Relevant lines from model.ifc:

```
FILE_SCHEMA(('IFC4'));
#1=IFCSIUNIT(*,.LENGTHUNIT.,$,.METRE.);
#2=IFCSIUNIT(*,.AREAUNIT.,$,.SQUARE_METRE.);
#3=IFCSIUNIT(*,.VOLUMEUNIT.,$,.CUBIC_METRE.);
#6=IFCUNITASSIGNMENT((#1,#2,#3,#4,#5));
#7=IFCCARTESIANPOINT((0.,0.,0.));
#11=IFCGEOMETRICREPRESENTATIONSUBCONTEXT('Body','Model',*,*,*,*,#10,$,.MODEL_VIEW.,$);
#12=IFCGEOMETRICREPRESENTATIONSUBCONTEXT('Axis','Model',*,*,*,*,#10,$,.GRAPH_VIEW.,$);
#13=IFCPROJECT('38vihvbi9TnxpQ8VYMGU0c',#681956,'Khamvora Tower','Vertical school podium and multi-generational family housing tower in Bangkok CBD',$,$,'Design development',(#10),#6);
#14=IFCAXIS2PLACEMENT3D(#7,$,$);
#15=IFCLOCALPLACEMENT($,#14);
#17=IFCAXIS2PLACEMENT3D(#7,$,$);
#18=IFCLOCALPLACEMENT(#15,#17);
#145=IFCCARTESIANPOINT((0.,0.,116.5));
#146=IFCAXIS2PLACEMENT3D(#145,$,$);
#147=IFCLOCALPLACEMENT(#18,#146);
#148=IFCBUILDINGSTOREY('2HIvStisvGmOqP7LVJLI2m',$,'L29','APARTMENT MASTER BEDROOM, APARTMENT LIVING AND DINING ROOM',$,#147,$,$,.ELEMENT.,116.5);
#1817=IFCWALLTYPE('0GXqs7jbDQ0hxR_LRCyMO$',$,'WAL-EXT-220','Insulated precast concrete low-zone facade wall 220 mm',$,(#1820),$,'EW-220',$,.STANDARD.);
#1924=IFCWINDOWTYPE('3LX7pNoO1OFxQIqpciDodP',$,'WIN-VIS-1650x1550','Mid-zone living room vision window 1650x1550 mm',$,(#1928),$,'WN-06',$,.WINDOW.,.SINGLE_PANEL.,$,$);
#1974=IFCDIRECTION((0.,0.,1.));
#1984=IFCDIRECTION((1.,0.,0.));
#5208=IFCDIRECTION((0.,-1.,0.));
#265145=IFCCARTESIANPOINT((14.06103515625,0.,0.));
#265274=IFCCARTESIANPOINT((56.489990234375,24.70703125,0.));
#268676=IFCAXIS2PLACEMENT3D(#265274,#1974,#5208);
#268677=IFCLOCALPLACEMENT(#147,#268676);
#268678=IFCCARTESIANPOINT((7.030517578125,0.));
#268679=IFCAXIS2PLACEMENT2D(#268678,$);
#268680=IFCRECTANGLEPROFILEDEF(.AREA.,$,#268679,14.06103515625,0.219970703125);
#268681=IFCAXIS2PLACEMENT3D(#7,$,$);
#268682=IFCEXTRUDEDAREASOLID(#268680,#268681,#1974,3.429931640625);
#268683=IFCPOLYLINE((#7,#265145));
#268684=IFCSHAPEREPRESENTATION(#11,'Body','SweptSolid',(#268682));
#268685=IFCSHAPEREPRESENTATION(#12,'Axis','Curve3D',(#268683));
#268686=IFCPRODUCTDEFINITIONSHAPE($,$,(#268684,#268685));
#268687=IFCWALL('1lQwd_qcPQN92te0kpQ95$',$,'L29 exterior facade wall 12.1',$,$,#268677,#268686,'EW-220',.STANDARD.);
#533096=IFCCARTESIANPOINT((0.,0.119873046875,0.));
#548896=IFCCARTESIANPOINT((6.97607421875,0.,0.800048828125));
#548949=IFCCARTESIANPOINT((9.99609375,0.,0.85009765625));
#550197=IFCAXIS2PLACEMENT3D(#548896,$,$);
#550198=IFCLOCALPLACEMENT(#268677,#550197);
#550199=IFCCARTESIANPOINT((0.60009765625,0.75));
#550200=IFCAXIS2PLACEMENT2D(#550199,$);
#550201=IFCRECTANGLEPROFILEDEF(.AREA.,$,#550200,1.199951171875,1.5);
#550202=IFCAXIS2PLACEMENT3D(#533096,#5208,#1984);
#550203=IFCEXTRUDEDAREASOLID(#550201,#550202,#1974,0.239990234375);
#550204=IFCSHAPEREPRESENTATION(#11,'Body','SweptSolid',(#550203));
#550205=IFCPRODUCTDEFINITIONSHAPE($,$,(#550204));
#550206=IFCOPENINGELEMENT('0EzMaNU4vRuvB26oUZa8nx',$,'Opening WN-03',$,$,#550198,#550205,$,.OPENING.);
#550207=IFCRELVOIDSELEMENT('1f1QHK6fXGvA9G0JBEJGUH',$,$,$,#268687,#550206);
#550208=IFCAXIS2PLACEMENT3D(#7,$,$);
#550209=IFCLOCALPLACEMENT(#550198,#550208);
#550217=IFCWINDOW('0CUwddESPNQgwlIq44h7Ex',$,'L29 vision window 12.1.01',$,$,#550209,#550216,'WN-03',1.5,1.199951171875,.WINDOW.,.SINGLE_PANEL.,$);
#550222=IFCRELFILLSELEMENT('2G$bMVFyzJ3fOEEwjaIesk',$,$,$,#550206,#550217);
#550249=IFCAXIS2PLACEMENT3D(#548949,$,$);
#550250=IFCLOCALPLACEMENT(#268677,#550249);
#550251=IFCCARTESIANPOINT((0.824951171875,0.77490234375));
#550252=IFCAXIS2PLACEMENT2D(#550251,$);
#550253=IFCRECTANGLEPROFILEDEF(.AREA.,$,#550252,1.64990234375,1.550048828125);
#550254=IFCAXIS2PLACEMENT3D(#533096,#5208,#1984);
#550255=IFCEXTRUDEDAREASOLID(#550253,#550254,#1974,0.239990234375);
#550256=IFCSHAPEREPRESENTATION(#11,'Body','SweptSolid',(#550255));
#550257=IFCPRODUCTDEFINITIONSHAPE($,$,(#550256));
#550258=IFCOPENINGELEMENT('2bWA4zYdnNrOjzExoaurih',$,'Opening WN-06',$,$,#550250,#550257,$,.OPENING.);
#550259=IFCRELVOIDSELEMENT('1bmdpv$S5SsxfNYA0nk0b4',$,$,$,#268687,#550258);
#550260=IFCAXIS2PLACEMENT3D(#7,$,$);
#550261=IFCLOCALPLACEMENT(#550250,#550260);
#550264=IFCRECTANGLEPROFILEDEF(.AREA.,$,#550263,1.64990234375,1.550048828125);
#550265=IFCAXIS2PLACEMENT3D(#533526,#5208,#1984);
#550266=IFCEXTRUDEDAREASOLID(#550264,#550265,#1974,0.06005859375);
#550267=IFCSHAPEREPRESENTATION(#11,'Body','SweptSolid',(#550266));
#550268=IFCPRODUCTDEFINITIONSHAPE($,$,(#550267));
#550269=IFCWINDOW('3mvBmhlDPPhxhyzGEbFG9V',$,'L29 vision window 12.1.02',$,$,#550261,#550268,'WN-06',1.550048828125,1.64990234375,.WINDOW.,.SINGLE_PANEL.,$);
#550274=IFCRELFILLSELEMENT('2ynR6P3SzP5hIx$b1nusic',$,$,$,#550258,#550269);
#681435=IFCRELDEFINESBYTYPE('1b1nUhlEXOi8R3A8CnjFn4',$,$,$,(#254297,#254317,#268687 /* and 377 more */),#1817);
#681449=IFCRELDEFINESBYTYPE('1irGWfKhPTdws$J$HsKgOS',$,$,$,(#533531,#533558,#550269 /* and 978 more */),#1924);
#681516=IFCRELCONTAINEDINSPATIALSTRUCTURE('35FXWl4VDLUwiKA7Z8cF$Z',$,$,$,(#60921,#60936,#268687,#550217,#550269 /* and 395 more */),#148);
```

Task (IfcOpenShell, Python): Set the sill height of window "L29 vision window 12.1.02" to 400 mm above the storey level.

```python
import numpy as np
import ifcopenshell
import ifcopenshell.api.geometry
import ifcopenshell.geom
import ifcopenshell.util.element
import ifcopenshell.util.placement
import ifcopenshell.util.shape
import ifcopenshell.util.unit

model = ifcopenshell.open("model.ifc")
unit_scale = ifcopenshell.util.unit.calculate_unit_scale(model)

window = model.by_guid("3mvBmhlDPPhxhyzGEbFG9V")
opening = window.FillsVoids[0].RelatingOpeningElement
storey = ifcopenshell.util.element.get_container(window, ifc_class="IfcBuildingStorey")
level = ifcopenshell.util.placement.get_local_placement(storey.ObjectPlacement)[2, 3]

# The opening's origin need not be at the sill, so measure its lowest point.
shape = ifcopenshell.geom.create_shape(ifcopenshell.geom.settings(), opening)
bottom = ifcopenshell.util.shape.get_shape_bottom_elevation(shape, shape.geometry) / unit_scale
dz = level + 0.4 / unit_scale - bottom

shift = np.array([0.0, 0.0, dz])
# The window is placed relative to its opening, so it follows when the opening moves.
matrix = ifcopenshell.util.placement.get_local_placement(opening.ObjectPlacement)
matrix[:3, 3] += shift
ifcopenshell.api.geometry.edit_object_placement(
    model, product=opening, matrix=matrix, is_si=False, should_transform_children=True
)

print(f"moved by {dz * unit_scale:+.3f} m")

model.write("model_v2.ifc")
```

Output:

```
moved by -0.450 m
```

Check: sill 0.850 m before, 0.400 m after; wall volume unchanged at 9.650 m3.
